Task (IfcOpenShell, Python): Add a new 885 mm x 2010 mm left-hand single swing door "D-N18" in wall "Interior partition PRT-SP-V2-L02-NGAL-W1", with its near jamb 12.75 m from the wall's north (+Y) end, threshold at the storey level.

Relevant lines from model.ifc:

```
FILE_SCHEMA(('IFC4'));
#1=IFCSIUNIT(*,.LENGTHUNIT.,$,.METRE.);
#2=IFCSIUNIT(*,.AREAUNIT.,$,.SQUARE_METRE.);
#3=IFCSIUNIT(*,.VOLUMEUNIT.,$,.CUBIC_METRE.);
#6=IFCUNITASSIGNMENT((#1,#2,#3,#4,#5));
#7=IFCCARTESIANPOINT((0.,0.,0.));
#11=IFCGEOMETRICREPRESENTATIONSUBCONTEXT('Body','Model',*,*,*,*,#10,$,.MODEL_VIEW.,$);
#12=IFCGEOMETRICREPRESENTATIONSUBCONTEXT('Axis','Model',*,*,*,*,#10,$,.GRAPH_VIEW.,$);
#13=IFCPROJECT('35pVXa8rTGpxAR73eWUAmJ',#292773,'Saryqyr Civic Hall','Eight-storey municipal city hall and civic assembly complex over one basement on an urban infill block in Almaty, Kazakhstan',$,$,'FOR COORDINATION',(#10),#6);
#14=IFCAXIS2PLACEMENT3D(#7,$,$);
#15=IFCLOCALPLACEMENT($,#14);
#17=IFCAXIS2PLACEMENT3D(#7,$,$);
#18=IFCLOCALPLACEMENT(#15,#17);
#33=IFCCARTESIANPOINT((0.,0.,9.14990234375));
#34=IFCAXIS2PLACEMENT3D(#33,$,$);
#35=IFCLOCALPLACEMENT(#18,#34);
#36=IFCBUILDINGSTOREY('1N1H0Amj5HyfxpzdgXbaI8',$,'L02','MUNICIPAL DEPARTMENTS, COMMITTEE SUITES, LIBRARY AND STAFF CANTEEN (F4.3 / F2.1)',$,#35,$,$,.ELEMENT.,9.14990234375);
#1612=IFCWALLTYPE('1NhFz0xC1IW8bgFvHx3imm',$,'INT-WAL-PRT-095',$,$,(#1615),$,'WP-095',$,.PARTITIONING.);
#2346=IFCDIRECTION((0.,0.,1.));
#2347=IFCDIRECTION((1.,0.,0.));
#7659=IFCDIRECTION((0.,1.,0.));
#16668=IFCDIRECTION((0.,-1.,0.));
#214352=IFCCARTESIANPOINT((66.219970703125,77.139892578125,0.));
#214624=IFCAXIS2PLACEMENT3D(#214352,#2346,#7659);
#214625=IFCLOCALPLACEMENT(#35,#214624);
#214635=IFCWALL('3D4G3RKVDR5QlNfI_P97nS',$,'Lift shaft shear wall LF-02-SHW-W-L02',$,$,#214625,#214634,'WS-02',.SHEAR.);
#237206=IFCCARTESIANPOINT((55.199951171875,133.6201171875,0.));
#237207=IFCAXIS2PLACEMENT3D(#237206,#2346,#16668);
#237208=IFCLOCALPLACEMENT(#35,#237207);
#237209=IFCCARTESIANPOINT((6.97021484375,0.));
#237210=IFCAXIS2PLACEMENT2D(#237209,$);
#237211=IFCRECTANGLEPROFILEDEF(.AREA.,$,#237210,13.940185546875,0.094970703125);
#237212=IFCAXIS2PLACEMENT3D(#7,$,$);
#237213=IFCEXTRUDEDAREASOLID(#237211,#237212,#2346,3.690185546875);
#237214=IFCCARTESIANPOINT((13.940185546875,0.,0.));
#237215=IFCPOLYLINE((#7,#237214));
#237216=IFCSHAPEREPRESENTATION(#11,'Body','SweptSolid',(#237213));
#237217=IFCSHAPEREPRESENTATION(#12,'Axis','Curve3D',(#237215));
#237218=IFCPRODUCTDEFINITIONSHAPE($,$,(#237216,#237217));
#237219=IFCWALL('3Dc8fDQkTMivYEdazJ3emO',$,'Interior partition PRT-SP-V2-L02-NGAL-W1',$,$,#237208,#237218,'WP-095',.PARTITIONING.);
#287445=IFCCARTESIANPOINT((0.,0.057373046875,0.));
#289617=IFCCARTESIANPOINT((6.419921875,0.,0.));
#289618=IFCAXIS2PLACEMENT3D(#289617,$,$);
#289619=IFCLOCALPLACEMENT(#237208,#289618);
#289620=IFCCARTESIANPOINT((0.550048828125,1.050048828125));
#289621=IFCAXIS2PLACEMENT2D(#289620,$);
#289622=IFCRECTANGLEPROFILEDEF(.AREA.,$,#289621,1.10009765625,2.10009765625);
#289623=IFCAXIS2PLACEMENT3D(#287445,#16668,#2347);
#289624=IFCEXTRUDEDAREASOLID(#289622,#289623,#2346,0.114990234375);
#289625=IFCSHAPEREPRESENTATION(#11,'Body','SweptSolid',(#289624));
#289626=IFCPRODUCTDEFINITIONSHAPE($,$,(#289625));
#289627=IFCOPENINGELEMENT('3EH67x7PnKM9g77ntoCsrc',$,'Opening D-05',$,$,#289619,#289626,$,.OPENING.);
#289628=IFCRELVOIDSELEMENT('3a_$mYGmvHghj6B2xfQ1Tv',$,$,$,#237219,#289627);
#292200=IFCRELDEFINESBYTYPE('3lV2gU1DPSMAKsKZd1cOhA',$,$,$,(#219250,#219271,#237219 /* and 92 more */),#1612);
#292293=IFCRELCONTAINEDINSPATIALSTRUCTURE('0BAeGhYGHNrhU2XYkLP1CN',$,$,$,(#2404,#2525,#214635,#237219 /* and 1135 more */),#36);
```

```python
import numpy as np
import ifcopenshell
import ifcopenshell.api.feature
import ifcopenshell.api.geometry
import ifcopenshell.api.root
import ifcopenshell.api.spatial
import ifcopenshell.geom
import ifcopenshell.util.element
import ifcopenshell.util.placement
import ifcopenshell.util.representation
import ifcopenshell.util.shape
import ifcopenshell.util.unit

model = ifcopenshell.open("model.ifc")
unit_scale = ifcopenshell.util.unit.calculate_unit_scale(model)
settings = ifcopenshell.geom.settings()


def volume(element):
    """Net volume in cubic metres, openings subtracted."""
    shape = ifcopenshell.geom.create_shape(settings, element)
    return ifcopenshell.util.shape.get_volume(shape.geometry)


wall = model.by_guid("3Dc8fDQkTMivYEdazJ3emO")
storey = ifcopenshell.util.element.get_container(wall, ifc_class="IfcBuildingStorey")
context = ifcopenshell.util.representation.get_context(model, "Model", "Body", "MODEL_VIEW")
before = volume(wall)

width, height, from_end, sill = 0.885, 2.01, 12.75, 0.0  # metres

# The wall runs along its own X axis, and the end named is its -X end.
wall_shape = ifcopenshell.geom.create_shape(settings, wall)
x, y, z = ifcopenshell.util.shape.get_vertices(wall_shape.geometry).T
start = x.min() + from_end
face, thickness = float(y.min()), float(y.max() - y.min())
wall_matrix = ifcopenshell.util.placement.get_local_placement(wall.ObjectPlacement)
level = ifcopenshell.util.placement.get_local_placement(storey.ObjectPlacement)[2, 3]


def in_wall(x, y):
    """Placement at x, y metres in the wall's axes, at sill height."""
    matrix = wall_matrix.copy()
    matrix[:, 3] = wall_matrix @ np.array([x / unit_scale, y / unit_scale, 0.0, 1.0])
    matrix[2, 3] = level + sill / unit_scale
    return matrix


# Opening: a box that overshoots both wall faces by 50 mm.
opening = ifcopenshell.api.root.create_entity(model, ifc_class="IfcOpeningElement", predefined_type="OPENING")
box = ifcopenshell.api.geometry.add_wall_representation(
    model, context=context, length=width, height=height, thickness=thickness + 0.1
)
ifcopenshell.api.geometry.assign_representation(model, product=opening, representation=box)
ifcopenshell.api.geometry.edit_object_placement(model, product=opening, matrix=in_wall(start, face - 0.05), is_si=False)
ifcopenshell.api.feature.add_feature(model, feature=opening, element=wall)

door = ifcopenshell.api.root.create_entity(model, ifc_class="IfcDoor", name="D-N18", predefined_type="DOOR")
door.OverallWidth, door.OverallHeight = width / unit_scale, height / unit_scale
door.OperationType = "SINGLE_SWING_LEFT"
body = ifcopenshell.api.geometry.add_door_representation(
    model,
    context=context,
    overall_width=door.OverallWidth,
    overall_height=door.OverallHeight,
    operation_type="SINGLE_SWING_LEFT",
    lining_properties={"LiningDepth": thickness / unit_scale, "ThresholdDepth": thickness / unit_scale},
)
ifcopenshell.api.geometry.assign_representation(model, product=door, representation=body)
ifcopenshell.api.spatial.assign_container(model, products=[door], relating_structure=storey)
ifcopenshell.api.feature.add_filling(model, opening=opening, element=door)

# The lining spans the wall, so the door starts at the wall face.
ifcopenshell.api.geometry.edit_object_placement(model, product=door, matrix=in_wall(start, face), is_si=False)

after = volume(wall)

print(f"wall volume {before:.3f} -> {after:.3f} m3")

model.write("model_updated.ifc")
```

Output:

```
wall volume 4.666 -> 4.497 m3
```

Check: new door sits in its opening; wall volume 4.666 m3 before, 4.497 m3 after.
